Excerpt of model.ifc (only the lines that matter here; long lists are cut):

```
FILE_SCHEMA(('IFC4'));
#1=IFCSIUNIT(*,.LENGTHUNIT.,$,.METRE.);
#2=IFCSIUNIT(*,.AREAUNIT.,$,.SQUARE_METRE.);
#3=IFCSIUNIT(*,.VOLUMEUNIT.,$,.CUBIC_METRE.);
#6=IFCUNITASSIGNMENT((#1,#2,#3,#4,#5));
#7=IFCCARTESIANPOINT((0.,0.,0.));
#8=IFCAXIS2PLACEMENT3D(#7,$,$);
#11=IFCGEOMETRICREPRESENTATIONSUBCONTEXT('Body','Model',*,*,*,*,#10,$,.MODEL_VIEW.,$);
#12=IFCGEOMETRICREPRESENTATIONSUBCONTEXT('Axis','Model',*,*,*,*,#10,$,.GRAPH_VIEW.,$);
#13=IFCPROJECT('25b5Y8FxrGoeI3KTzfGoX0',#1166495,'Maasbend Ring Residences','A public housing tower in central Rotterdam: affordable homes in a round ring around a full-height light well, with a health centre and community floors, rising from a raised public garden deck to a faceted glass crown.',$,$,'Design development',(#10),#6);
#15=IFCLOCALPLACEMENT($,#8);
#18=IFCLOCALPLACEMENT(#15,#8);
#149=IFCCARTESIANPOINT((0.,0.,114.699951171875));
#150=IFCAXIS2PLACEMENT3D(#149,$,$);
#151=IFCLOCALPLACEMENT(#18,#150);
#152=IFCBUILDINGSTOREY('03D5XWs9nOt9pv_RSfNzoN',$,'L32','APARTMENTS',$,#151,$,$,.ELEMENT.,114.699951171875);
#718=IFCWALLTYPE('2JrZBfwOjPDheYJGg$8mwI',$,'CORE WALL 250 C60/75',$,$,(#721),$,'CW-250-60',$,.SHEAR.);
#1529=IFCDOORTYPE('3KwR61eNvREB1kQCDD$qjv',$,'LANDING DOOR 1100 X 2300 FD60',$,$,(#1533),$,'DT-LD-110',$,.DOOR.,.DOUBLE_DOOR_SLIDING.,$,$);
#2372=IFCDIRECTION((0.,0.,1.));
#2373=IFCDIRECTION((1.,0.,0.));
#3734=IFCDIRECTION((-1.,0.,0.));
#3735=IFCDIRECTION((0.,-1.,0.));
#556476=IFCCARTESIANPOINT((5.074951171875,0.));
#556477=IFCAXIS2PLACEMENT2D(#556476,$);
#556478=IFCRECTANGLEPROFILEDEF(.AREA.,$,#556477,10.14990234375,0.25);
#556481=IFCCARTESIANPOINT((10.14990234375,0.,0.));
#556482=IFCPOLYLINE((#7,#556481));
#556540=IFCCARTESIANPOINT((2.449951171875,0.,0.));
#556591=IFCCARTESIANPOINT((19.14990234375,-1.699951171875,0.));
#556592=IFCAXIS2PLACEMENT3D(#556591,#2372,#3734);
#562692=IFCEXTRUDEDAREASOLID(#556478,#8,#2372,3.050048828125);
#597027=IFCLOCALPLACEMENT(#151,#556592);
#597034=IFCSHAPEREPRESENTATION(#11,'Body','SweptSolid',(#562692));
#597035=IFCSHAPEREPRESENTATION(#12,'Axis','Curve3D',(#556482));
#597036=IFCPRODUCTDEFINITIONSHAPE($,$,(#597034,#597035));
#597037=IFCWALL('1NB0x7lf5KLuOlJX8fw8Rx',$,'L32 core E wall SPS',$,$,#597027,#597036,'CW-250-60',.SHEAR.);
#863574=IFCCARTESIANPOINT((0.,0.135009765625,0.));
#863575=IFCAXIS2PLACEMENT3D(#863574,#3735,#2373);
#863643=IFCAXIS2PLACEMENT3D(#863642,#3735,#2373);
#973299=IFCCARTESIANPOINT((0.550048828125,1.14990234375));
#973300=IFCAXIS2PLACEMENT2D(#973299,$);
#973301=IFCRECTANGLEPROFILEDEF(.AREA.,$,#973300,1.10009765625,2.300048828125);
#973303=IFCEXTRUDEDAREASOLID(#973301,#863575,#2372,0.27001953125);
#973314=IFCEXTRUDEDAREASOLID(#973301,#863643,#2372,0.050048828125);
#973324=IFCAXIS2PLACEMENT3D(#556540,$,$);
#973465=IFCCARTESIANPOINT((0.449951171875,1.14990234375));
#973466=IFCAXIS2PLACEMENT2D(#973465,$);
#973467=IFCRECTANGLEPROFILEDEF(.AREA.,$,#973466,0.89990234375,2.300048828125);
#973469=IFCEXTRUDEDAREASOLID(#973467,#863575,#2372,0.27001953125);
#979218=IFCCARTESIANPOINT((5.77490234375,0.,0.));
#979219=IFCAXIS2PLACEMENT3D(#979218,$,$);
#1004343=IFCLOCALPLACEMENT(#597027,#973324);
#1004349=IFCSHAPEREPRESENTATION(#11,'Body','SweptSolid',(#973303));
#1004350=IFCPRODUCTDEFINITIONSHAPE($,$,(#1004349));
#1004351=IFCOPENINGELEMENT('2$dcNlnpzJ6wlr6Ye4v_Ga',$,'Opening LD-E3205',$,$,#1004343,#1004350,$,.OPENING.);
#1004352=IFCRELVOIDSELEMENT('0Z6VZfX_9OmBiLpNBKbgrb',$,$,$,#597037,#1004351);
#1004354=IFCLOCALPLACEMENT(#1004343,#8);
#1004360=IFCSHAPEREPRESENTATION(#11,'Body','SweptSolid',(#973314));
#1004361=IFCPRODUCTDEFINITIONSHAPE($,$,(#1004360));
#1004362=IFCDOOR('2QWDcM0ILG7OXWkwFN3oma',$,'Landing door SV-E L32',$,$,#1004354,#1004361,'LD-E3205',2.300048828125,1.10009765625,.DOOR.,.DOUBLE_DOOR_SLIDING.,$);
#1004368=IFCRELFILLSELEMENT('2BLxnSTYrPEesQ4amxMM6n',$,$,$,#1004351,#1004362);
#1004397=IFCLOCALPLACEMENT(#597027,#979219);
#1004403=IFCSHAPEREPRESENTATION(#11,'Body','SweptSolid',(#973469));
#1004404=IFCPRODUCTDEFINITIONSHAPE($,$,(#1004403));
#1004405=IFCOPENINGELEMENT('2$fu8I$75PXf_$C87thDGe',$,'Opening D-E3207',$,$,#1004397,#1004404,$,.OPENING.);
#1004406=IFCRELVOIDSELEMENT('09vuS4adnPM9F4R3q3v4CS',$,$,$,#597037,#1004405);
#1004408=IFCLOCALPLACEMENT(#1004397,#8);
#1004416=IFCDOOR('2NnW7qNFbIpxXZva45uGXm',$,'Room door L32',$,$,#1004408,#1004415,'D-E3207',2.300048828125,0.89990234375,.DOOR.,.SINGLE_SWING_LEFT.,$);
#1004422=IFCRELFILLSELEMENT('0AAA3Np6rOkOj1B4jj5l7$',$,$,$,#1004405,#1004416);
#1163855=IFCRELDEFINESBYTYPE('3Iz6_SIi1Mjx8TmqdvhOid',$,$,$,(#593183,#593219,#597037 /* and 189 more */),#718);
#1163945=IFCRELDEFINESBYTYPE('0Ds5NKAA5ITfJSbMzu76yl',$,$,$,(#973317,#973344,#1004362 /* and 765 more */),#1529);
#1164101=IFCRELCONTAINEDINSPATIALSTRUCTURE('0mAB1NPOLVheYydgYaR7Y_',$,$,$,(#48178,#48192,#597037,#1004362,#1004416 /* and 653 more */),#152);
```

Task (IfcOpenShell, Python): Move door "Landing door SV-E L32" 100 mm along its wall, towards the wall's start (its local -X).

```python
import ifcopenshell
import ifcopenshell.api.geometry
import ifcopenshell.util.placement

model = ifcopenshell.open("model.ifc")

door = model.by_guid("2QWDcM0ILG7OXWkwFN3oma")
opening = door.FillsVoids[0].RelatingOpeningElement
wall = opening.VoidsElements[0].RelatingBuildingElement

wall_matrix = ifcopenshell.util.placement.get_local_placement(wall.ObjectPlacement)
shift = wall_matrix[:3, 0] * -0.1
before = ifcopenshell.util.placement.get_local_placement(door.ObjectPlacement)[:3, 3].copy()

# The door is placed relative to its opening, so it follows when the opening moves.
matrix = ifcopenshell.util.placement.get_local_placement(opening.ObjectPlacement)
matrix[:3, 3] += shift
ifcopenshell.api.geometry.edit_object_placement(
    model, product=opening, matrix=matrix, is_si=False, should_transform_children=True
)

after = ifcopenshell.util.placement.get_local_placement(door.ObjectPlacement)[:3, 3]
print("door moved by", (after - before).round(3) + 0.0)

model.write("model-out.ifc")
```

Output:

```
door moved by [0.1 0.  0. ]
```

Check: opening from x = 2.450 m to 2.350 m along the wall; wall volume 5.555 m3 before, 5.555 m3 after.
